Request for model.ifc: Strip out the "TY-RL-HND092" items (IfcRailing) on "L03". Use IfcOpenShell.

First a look at what the model holds.

```python
import ifcopenshell
import ifcopenshell.util.element

model = ifcopenshell.open("model.ifc")
print(model.schema)
storey = next(s for s in model.by_type("IfcBuildingStorey") if s.Name == "L03")
railings = [e for e in ifcopenshell.util.element.get_decomposition(storey) if e.is_a("IfcRailing")]
seen = {}
for e in railings:
    element_type = ifcopenshell.util.element.get_type(e)
    name = element_type.Name if element_type not in (None, e) else None
    seen[name] = seen.get(name, 0) + 1
for name, count in sorted(seen.items(), key=str):
    print(count, "x", name)
```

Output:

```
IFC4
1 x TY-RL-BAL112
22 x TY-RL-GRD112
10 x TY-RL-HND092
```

```python
import ifcopenshell
import ifcopenshell.api.root
import ifcopenshell.util.element

model = ifcopenshell.open("model.ifc")

storey = next(s for s in model.by_type("IfcBuildingStorey") if s.Name == "L03")
railings = [e for e in ifcopenshell.util.element.get_decomposition(storey) if e.is_a("IfcRailing")]
targets = [e for e in railings if (t := ifcopenshell.util.element.get_type(e)) not in (None, e) and t.Name == "TY-RL-HND092"]

for e in targets:
    ifcopenshell.api.root.remove_product(model, product=e)
print(len(targets), "removed")

model.write("model_updated.ifc")
```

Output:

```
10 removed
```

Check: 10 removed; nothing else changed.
